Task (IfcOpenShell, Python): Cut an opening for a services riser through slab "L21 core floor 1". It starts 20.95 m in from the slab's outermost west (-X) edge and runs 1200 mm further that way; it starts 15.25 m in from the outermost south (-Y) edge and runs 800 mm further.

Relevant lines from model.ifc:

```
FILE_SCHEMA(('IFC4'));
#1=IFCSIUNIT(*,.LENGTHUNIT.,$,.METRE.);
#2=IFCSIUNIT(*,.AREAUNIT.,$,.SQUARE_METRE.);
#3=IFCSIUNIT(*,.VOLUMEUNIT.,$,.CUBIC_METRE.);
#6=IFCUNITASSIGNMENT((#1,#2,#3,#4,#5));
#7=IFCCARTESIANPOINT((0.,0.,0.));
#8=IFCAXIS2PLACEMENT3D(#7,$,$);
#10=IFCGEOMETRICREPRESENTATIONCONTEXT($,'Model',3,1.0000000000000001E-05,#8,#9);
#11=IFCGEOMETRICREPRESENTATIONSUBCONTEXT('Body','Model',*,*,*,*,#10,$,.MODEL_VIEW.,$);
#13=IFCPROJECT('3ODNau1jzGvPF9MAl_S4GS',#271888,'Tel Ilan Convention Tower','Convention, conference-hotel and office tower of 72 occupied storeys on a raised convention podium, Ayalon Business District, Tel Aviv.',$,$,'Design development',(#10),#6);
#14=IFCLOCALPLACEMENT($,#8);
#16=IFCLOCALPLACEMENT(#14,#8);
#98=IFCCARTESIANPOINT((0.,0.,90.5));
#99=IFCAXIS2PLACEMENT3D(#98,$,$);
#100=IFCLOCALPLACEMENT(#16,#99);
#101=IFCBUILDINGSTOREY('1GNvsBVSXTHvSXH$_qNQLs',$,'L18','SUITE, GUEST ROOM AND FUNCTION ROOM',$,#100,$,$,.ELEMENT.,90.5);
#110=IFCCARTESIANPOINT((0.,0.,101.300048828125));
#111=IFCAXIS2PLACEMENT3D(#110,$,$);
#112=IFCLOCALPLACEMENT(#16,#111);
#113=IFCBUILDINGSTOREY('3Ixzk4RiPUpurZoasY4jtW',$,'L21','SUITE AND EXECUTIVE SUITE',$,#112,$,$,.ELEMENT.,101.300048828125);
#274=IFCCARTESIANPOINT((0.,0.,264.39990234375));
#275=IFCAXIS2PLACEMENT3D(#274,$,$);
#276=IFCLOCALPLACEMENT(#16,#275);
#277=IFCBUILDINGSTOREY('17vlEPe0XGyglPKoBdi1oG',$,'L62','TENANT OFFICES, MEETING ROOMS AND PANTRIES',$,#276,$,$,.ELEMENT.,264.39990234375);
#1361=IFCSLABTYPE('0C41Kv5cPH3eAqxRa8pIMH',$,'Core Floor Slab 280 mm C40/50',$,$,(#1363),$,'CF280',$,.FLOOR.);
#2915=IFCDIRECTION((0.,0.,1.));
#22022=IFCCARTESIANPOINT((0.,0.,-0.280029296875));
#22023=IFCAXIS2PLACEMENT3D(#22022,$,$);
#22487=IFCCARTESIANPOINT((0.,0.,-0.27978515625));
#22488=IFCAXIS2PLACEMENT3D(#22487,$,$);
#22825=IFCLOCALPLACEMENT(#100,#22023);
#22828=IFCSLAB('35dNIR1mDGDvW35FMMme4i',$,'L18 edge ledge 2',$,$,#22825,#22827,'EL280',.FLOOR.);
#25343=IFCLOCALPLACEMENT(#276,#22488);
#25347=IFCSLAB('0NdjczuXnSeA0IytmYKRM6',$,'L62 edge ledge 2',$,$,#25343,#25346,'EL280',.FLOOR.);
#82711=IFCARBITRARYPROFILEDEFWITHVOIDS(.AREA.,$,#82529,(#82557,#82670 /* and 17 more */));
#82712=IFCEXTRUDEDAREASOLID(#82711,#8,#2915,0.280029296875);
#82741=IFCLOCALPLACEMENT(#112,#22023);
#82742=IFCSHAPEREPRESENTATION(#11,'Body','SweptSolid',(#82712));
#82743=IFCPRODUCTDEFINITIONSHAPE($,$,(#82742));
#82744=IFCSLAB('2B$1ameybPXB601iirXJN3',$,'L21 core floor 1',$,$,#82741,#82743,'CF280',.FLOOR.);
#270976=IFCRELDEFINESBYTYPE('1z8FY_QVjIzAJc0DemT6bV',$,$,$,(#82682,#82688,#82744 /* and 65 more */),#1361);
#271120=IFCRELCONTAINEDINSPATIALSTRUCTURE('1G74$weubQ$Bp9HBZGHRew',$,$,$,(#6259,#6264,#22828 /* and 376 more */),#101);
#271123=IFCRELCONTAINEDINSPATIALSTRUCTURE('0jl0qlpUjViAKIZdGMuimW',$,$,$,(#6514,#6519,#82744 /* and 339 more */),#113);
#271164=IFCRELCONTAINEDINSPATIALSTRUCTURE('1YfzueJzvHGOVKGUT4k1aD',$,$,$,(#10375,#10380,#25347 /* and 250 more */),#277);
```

```python
import numpy as np
import ifcopenshell
import ifcopenshell.api.feature
import ifcopenshell.api.geometry
import ifcopenshell.api.root
import ifcopenshell.geom
import ifcopenshell.util.placement
import ifcopenshell.util.representation
import ifcopenshell.util.shape
import ifcopenshell.util.unit

model = ifcopenshell.open("model.ifc")
unit_scale = ifcopenshell.util.unit.calculate_unit_scale(model)
settings = ifcopenshell.geom.settings()


def volume(element):
    """Net volume in cubic metres, openings subtracted."""
    shape = ifcopenshell.geom.create_shape(settings, element)
    return ifcopenshell.util.shape.get_volume(shape.geometry)


slab = model.by_id(82744)
before = volume(slab)

# Extent in the slab's own axes, in metres. The edges named are its -X and -Y sides.
slab_shape = ifcopenshell.geom.create_shape(settings, slab)
vertices = ifcopenshell.util.shape.get_vertices(slab_shape.geometry)
x_min, y_min, bottom = vertices.min(axis=0)
top = vertices[:, 2].max()

opening = ifcopenshell.api.root.create_entity(model, ifc_class="IfcOpeningElement", name="Services riser opening", predefined_type="OPENING")
context = ifcopenshell.util.representation.get_context(model, "Model", "Body", "MODEL_VIEW")
width, depth = 1.2, 0.8
outline = [(0.0, 0.0), (width, 0.0), (width, depth), (0.0, depth), (0.0, 0.0)]
# Overshoot both faces by 50 mm so the cut is clean.
shape = ifcopenshell.api.geometry.add_slab_representation(
    model, context=context, depth=top - bottom + 0.1, polyline=outline
)
ifcopenshell.api.geometry.assign_representation(model, product=opening, representation=shape)

matrix = ifcopenshell.util.placement.get_local_placement(slab.ObjectPlacement)
matrix[:, 3] = matrix @ np.append(np.array([x_min + 20.95, y_min + 15.25, bottom - 0.05]) / unit_scale, 1.0)
ifcopenshell.api.geometry.edit_object_placement(model, product=opening, matrix=matrix, is_si=False)
ifcopenshell.api.feature.add_feature(model, feature=opening, element=slab)

after = volume(slab)

print(f"slab volume {before:.3f} -> {after:.3f} m3")

model.write("model_rev.ifc")
```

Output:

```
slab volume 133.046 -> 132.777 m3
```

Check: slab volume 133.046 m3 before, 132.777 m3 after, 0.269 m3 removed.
